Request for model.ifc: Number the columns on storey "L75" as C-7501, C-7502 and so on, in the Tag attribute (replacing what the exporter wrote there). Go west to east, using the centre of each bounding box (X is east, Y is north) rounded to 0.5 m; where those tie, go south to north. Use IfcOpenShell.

First a look at what the model holds.

```python
import ifcopenshell
import ifcopenshell.util.element
import ifcopenshell.util.placement

model = ifcopenshell.open("model.ifc")
print(model.schema)
storey = next(s for s in model.by_type("IfcBuildingStorey") if s.Name == "L75")
columns = [e for e in ifcopenshell.util.element.get_decomposition(storey) if e.is_a("IfcColumn")]
for e in sorted(columns, key=lambda e: e.id()):
    origin = ifcopenshell.util.placement.get_local_placement(e.ObjectPlacement)[:3, 3]
    print(e.id(), e.Tag, e.Name, origin.round(2) + 0.0, sep=" | ")
```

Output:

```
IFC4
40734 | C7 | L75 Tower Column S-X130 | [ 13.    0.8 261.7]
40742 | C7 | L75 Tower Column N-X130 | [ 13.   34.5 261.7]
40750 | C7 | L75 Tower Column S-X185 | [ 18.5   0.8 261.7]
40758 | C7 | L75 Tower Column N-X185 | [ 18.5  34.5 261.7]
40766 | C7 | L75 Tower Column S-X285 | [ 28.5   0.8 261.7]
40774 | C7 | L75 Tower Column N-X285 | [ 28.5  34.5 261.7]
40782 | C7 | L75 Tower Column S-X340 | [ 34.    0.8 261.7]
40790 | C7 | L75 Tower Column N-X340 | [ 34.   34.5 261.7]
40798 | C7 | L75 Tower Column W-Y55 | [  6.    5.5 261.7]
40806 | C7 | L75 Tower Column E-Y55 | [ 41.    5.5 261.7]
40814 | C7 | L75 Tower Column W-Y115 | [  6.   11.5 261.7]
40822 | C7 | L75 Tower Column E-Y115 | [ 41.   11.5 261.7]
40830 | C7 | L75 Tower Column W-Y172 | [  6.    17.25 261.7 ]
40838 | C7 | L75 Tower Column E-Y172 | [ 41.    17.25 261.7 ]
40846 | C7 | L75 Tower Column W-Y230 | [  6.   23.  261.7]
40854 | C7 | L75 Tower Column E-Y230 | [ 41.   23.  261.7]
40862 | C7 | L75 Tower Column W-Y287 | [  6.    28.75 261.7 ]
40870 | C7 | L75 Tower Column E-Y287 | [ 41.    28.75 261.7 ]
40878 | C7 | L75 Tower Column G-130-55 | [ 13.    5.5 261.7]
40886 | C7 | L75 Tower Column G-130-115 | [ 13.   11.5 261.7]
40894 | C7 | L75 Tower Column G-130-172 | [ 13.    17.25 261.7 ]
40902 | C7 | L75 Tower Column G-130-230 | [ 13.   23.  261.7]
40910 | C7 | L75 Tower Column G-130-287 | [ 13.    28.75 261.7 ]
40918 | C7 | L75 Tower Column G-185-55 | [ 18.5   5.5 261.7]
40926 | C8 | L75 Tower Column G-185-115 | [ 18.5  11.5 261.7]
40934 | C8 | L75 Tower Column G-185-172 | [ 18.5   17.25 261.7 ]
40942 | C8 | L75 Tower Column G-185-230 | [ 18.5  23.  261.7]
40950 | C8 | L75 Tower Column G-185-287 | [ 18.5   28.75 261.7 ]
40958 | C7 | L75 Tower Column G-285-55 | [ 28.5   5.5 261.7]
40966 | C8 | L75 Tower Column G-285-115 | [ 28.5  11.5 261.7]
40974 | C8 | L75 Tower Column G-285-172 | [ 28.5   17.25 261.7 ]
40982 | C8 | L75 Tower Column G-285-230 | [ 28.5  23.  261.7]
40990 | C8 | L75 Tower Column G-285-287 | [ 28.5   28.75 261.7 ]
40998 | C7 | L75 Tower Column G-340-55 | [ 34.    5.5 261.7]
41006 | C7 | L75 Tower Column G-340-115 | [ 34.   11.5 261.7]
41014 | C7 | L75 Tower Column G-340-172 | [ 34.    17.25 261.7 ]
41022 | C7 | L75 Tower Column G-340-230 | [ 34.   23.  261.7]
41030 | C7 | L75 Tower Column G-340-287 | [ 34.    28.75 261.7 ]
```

```python
import ifcopenshell
import ifcopenshell.geom
import ifcopenshell.util.element
import ifcopenshell.util.shape

model = ifcopenshell.open("model.ifc")
settings = ifcopenshell.geom.settings()
settings.set("use-world-coords", True)


def centre(element):
    shape = ifcopenshell.geom.create_shape(settings, element)
    return ifcopenshell.util.shape.get_bbox_centroid(shape.geometry)


storey = next(s for s in model.by_type("IfcBuildingStorey") if s.Name == "L75")
columns = [e for e in ifcopenshell.util.element.get_decomposition(storey) if e.is_a("IfcColumn")]

# Insertion points can sit at a corner or the storey origin, so sort by the geometry (in metres).
centres = {e: centre(e) for e in columns}
columns.sort(key=lambda e: (round(centres[e][0] / 0.5), centres[e][1]))

for i, e in enumerate(columns, start=1):
    number = f"C-75{i:02d}"
    e.Tag = number
    print(e.id(), number)

model.write("model_rev.ifc")
```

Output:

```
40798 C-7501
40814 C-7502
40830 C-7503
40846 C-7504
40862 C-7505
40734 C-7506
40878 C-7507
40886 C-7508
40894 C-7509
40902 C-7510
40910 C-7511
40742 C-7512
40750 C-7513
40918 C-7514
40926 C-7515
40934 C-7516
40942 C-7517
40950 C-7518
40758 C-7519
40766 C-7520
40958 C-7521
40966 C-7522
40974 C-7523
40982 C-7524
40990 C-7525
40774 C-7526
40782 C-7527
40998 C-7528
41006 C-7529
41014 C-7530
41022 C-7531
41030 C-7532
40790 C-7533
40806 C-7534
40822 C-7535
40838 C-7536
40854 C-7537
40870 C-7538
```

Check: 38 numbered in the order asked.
